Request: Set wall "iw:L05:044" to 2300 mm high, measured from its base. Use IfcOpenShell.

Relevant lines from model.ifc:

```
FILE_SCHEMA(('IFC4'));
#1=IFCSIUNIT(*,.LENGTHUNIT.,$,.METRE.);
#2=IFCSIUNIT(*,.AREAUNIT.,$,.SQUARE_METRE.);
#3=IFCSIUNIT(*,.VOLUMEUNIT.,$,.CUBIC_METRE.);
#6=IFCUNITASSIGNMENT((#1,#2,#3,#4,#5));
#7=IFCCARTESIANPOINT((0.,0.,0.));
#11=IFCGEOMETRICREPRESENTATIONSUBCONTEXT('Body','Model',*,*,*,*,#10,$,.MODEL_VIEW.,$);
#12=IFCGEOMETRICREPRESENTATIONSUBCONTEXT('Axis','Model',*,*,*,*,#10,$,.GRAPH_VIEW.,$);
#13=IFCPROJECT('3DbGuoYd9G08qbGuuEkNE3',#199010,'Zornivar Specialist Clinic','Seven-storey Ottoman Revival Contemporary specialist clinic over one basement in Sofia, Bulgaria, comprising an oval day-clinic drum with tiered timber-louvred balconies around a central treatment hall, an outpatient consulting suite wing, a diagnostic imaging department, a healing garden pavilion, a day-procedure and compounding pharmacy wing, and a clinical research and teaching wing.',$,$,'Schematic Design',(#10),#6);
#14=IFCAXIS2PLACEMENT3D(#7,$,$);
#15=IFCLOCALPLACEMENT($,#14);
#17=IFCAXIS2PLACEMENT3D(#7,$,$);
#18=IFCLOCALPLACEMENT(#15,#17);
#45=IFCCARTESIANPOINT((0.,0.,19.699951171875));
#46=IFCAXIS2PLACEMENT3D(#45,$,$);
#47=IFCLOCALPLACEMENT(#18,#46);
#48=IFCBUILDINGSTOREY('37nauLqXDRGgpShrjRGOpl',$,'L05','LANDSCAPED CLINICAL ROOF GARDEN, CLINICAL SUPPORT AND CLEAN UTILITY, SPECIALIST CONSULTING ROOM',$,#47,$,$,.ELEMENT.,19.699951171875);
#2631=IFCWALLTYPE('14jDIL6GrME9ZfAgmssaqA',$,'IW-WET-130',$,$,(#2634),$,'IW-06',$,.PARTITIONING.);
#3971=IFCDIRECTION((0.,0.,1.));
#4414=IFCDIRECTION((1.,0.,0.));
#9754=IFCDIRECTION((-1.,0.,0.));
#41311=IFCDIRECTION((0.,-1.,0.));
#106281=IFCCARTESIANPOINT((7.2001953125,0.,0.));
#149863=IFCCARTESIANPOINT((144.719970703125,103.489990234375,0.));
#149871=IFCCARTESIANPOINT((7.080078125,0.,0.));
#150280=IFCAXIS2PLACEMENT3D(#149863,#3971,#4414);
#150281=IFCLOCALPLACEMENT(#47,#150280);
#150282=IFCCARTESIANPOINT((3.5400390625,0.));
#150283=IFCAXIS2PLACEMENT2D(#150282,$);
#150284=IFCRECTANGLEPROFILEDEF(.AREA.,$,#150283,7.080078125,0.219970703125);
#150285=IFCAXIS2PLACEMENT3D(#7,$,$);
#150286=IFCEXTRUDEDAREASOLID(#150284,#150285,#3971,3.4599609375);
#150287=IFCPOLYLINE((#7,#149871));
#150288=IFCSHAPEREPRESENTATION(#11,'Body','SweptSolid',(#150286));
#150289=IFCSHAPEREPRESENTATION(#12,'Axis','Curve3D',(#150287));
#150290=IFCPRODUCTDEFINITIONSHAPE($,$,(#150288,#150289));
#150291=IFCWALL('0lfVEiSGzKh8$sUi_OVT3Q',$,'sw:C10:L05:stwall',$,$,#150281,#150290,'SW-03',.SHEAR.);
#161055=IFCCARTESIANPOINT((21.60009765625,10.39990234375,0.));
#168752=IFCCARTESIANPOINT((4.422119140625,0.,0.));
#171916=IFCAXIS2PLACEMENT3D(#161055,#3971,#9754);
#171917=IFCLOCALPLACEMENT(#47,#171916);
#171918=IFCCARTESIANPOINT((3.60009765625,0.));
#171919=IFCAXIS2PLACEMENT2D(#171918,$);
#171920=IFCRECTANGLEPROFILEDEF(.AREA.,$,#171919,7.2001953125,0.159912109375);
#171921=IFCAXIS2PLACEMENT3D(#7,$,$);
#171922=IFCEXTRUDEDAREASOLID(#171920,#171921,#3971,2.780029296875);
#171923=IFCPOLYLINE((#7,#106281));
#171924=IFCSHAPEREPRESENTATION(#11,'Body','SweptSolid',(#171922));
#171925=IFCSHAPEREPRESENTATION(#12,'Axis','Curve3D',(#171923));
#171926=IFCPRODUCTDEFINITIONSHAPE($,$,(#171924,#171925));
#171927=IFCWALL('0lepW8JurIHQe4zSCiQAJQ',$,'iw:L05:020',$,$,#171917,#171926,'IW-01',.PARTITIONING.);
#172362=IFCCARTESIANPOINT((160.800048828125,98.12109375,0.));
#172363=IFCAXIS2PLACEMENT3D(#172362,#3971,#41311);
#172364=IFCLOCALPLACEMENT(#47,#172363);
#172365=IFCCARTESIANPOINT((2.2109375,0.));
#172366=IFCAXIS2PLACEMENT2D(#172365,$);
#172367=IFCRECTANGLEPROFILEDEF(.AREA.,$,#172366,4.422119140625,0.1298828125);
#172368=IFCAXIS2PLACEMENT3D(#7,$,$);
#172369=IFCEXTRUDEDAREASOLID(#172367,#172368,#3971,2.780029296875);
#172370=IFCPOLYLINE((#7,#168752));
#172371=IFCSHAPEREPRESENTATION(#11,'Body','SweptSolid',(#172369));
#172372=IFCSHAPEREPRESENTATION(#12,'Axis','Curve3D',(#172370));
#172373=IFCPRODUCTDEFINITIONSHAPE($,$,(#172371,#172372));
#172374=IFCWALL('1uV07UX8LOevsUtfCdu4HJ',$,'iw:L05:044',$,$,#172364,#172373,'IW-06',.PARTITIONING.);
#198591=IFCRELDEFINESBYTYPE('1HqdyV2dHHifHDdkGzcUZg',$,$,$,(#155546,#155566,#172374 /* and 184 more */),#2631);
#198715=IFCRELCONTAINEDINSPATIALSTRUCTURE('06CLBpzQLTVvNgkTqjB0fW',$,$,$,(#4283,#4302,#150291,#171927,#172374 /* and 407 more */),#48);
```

```python
import ifcopenshell
import ifcopenshell.geom
import ifcopenshell.util.representation
import ifcopenshell.util.shape

model = ifcopenshell.open("model.ifc")
settings = ifcopenshell.geom.settings()


def volume(element):
    """Net volume in cubic metres, openings subtracted."""
    shape = ifcopenshell.geom.create_shape(settings, element)
    return ifcopenshell.util.shape.get_volume(shape.geometry)


wall = model.by_guid("1uV07UX8LOevsUtfCdu4HJ")
before = volume(wall)

body = ifcopenshell.util.representation.get_representation(wall, "Model", "Body")
solid = body.Items[0]
old_height = solid.Depth
solid.Depth = 2.3
after = volume(wall)

print(f"height {old_height:g} -> {solid.Depth:g}, volume {before:.3f} -> {after:.3f} m3")

model.write("model_rev.ifc")
```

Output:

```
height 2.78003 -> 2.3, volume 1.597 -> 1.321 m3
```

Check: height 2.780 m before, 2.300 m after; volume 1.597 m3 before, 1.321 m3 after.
